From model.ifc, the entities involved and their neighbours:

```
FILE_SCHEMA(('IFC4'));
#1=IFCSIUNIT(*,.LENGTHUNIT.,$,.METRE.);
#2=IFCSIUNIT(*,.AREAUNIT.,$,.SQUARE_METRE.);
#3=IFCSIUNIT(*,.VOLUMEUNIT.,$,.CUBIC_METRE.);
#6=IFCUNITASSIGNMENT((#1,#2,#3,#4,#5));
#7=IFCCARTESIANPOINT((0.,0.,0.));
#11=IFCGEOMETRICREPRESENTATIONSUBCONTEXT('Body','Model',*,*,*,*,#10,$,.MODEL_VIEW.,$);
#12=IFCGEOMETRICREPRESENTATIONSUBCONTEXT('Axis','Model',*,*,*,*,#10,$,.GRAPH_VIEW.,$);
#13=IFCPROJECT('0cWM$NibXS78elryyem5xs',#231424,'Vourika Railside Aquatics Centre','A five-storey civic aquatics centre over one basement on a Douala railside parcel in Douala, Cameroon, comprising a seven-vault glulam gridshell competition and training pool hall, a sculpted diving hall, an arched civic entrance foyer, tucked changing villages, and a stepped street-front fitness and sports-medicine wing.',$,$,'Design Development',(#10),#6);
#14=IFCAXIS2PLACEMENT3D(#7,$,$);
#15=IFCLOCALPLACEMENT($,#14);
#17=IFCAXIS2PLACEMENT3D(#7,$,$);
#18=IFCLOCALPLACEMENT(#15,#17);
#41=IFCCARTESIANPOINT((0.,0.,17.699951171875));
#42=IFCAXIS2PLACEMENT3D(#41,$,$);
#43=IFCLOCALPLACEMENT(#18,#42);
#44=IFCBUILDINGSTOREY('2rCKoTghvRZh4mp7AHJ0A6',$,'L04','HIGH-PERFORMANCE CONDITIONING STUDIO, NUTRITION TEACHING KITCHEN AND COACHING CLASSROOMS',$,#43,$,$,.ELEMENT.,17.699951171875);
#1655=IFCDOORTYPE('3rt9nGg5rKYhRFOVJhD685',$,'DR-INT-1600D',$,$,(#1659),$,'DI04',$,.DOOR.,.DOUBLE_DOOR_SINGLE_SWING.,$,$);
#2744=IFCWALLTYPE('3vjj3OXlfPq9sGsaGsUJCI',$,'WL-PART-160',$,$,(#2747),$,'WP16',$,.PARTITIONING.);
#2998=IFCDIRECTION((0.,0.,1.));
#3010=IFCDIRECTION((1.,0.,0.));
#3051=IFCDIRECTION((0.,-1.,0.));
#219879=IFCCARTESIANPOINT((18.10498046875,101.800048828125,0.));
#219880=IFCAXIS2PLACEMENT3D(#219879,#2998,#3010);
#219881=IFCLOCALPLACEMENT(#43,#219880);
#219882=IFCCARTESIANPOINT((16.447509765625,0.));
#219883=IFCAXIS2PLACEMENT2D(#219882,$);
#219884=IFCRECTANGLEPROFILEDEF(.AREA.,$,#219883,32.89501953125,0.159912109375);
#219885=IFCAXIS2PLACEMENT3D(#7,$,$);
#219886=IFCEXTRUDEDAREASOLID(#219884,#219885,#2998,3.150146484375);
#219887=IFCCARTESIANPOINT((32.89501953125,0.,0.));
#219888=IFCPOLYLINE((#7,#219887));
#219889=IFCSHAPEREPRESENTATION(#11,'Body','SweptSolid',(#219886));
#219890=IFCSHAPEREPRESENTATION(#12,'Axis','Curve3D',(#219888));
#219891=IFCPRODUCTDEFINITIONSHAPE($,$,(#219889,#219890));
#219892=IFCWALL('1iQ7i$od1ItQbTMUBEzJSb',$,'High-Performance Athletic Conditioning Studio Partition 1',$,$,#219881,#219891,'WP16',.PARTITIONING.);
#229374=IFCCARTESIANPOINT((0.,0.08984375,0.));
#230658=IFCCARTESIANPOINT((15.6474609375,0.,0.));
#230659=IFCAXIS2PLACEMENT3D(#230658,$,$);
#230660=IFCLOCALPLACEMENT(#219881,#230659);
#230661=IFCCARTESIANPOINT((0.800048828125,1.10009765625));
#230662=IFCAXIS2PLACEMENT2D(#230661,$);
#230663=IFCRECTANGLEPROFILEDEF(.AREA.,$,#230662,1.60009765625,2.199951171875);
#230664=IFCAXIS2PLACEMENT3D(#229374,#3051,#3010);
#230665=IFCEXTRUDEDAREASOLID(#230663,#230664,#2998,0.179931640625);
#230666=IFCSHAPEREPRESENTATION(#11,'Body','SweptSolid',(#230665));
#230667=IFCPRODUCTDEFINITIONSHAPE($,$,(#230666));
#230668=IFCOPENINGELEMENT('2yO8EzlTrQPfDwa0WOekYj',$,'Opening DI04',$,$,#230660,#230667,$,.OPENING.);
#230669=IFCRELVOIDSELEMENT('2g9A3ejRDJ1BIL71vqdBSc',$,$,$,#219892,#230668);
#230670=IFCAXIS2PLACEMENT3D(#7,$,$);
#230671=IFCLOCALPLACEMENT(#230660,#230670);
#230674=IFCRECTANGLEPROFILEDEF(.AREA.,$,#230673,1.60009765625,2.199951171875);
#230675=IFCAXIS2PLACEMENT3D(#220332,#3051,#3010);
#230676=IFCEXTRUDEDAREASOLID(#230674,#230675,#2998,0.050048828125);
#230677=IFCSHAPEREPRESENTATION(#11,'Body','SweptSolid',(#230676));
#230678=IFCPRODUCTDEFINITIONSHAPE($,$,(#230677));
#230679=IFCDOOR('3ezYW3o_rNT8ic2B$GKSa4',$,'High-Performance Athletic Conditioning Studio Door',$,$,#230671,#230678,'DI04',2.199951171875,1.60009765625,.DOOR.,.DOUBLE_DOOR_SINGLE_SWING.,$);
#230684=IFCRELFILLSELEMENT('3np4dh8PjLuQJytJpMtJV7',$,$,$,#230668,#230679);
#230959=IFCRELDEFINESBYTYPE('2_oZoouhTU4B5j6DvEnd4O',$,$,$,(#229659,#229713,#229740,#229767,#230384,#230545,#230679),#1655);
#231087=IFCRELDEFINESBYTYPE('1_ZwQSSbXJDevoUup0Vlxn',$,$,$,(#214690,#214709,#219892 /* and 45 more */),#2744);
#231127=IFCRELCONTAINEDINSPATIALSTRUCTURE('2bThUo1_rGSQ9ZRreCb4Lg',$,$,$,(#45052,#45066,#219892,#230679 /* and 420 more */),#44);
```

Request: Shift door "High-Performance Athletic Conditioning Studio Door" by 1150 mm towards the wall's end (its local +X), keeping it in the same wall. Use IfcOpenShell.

```python
import ifcopenshell
import ifcopenshell.api.geometry
import ifcopenshell.util.placement
import ifcopenshell.util.unit

model = ifcopenshell.open("model.ifc")
unit_scale = ifcopenshell.util.unit.calculate_unit_scale(model)

door = model.by_guid("3ezYW3o_rNT8ic2B$GKSa4")
opening = door.FillsVoids[0].RelatingOpeningElement
wall = opening.VoidsElements[0].RelatingBuildingElement

wall_matrix = ifcopenshell.util.placement.get_local_placement(wall.ObjectPlacement)
shift = wall_matrix[:3, 0] * 1.15 / unit_scale
before = ifcopenshell.util.placement.get_local_placement(door.ObjectPlacement)[:3, 3].copy()

# The door is placed relative to its opening, so it follows when the opening moves.
matrix = ifcopenshell.util.placement.get_local_placement(opening.ObjectPlacement)
matrix[:3, 3] += shift
ifcopenshell.api.geometry.edit_object_placement(
    model, product=opening, matrix=matrix, is_si=False, should_transform_children=True
)

after = ifcopenshell.util.placement.get_local_placement(door.ObjectPlacement)[:3, 3]
print("door moved by", (after - before).round(3) + 0.0)

model.write("model_updated.ifc")
```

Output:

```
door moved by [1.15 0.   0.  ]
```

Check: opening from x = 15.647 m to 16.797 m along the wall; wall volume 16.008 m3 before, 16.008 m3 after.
